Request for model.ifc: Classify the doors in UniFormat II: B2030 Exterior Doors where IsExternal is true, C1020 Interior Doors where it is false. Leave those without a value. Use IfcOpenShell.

First a look at what the model holds.

```python
import ifcopenshell
import ifcopenshell.util.element

model = ifcopenshell.open("model.ifc")
print(model.schema)
print("classifications:", [c.Name for c in model.by_type("IfcClassification")])
values = [ifcopenshell.util.element.get_pset(e, "Pset_DoorCommon", "IsExternal") for e in model.by_type("IfcDoor")]
for value in (True, False, None):
    print("IsExternal", value, values.count(value))
```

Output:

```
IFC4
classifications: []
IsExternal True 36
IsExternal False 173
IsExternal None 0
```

```python
import ifcopenshell
import ifcopenshell.api.classification
import ifcopenshell.util.element

model = ifcopenshell.open("model.ifc")

system = ifcopenshell.api.classification.add_classification(model, classification="UniFormat II")

doors = model.by_type("IfcDoor")
external = {e: ifcopenshell.util.element.get_pset(e, "Pset_DoorCommon", "IsExternal") for e in doors}
for flag, code, name in ((True, "B2030", "Exterior Doors"), (False, "C1020", "Interior Doors")):
    products = [e for e in doors if external[e] is flag]
    ifcopenshell.api.classification.add_reference(
        model, products=products, classification=system, identification=code, name=name
    )
    print(code, len(products))

model.write("model-out.ifc")
```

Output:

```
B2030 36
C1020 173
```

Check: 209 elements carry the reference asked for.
